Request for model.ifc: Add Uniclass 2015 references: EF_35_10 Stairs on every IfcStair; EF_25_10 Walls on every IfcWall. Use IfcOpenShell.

First a look at what the model holds.

```python
import ifcopenshell

model = ifcopenshell.open("model.ifc")
print(model.schema)
print("classifications:", [c.Name for c in model.by_type("IfcClassification")])
for ifc_class in ("IfcDoor", "IfcRoof", "IfcStair", "IfcWall", "IfcWindow"):
    print(ifc_class, len(model.by_type(ifc_class)))
```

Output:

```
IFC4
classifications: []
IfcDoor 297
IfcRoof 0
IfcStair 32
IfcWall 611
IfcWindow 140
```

```python
import ifcopenshell
import ifcopenshell.api.classification

model = ifcopenshell.open("model.ifc")

system = ifcopenshell.api.classification.add_classification(model, classification="Uniclass 2015")

codes = {
    "IfcStair": ("EF_35_10", "Stairs"),
    "IfcWall": ("EF_25_10", "Walls"),
}
for ifc_class, (code, name) in codes.items():
    products = model.by_type(ifc_class)
    ifcopenshell.api.classification.add_reference(
        model, products=products, classification=system, identification=code, name=name
    )
    print(code, len(products))

model.write("model_v2.ifc")
```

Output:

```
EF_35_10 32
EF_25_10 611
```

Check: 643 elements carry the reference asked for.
